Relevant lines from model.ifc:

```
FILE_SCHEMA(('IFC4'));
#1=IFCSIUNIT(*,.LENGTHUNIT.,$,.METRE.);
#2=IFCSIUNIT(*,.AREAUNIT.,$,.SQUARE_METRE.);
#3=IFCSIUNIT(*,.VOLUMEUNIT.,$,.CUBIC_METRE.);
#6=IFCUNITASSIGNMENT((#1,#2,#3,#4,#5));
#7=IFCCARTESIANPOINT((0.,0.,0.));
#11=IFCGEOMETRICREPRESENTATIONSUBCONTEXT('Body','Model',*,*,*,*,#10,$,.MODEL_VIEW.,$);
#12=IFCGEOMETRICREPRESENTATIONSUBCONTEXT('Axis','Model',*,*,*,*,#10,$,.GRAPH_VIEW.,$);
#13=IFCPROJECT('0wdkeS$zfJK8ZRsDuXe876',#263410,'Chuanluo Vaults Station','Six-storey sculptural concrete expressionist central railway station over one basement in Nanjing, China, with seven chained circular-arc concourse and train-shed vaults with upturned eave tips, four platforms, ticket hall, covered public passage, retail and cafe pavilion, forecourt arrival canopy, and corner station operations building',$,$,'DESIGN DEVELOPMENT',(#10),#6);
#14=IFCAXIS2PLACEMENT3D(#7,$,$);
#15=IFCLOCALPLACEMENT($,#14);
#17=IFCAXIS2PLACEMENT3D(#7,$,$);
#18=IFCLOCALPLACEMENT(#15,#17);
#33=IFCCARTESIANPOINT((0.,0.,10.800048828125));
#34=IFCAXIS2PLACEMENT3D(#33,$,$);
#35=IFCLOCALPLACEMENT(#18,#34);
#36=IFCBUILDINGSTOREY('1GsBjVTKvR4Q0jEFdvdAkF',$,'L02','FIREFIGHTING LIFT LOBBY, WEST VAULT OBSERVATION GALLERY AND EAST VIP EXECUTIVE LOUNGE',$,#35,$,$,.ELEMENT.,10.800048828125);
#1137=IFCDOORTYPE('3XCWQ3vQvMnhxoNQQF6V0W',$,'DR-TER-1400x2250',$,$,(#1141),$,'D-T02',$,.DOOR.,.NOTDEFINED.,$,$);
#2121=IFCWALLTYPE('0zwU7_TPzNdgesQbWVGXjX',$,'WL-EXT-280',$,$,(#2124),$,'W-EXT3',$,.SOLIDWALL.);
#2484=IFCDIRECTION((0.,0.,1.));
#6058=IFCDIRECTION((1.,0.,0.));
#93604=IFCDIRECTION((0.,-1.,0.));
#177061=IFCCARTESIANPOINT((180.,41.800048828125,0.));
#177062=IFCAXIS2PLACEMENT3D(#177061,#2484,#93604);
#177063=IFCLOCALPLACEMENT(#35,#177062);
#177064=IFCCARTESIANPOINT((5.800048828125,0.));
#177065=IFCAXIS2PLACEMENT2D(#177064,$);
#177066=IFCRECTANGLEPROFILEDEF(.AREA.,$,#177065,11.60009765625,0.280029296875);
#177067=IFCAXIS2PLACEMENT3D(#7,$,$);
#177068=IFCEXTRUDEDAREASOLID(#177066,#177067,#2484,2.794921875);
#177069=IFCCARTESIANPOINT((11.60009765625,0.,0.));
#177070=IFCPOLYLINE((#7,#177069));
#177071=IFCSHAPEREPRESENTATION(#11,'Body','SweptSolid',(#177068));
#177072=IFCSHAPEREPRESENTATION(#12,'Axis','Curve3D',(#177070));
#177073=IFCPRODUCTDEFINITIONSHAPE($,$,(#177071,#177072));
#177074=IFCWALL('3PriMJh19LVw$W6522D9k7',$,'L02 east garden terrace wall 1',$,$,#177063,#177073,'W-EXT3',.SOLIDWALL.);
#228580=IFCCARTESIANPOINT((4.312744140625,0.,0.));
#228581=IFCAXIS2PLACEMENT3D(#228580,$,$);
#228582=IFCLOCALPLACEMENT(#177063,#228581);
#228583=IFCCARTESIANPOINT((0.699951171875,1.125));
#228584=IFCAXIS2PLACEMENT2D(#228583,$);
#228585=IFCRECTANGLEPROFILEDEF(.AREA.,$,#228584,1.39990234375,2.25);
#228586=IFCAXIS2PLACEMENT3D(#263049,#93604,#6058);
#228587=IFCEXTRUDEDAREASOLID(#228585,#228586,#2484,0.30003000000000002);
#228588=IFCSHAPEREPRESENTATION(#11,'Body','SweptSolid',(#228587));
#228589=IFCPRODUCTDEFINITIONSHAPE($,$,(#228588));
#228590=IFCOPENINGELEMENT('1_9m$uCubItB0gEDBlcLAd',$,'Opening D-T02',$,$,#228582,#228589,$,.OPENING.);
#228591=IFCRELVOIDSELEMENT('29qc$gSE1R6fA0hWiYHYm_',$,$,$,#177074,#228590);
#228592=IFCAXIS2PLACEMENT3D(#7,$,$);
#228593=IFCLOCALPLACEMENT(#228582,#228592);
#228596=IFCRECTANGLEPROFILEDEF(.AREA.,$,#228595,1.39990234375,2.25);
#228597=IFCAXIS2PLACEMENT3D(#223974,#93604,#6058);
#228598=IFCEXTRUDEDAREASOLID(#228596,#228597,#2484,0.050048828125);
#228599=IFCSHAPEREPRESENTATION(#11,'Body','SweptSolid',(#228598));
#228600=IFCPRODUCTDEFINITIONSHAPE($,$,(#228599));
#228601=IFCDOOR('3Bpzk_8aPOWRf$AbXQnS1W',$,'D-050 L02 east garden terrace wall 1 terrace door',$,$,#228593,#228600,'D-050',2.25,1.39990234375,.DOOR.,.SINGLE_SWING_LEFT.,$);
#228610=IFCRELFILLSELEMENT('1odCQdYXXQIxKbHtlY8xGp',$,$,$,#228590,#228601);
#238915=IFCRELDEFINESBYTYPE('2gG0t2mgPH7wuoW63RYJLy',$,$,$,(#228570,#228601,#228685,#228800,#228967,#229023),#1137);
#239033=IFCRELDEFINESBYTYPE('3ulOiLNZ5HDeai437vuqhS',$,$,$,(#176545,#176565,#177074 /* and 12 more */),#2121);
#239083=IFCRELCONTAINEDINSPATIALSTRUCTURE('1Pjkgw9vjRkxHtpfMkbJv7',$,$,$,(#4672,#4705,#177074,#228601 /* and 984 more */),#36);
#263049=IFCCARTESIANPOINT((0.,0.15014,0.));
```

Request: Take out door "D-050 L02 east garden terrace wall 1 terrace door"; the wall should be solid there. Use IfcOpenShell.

```python
import ifcopenshell
import ifcopenshell.api.feature
import ifcopenshell.api.root
import ifcopenshell.geom
import ifcopenshell.util.shape

model = ifcopenshell.open("model.ifc")
settings = ifcopenshell.geom.settings()


def volume(element):
    """Net volume in cubic metres, openings subtracted."""
    shape = ifcopenshell.geom.create_shape(settings, element)
    return ifcopenshell.util.shape.get_volume(shape.geometry)


door = model.by_guid("3Bpzk_8aPOWRf$AbXQnS1W")
opening = door.FillsVoids[0].RelatingOpeningElement
wall = opening.VoidsElements[0].RelatingBuildingElement
before = volume(wall)

ifcopenshell.api.root.remove_product(model, product=door)
ifcopenshell.api.feature.remove_feature(model, feature=opening)

after = volume(wall)

print(f"wall volume {before:.3f} -> {after:.3f} m3")

model.write("model-out.ifc")
```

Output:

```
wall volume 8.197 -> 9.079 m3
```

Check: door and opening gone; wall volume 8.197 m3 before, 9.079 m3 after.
